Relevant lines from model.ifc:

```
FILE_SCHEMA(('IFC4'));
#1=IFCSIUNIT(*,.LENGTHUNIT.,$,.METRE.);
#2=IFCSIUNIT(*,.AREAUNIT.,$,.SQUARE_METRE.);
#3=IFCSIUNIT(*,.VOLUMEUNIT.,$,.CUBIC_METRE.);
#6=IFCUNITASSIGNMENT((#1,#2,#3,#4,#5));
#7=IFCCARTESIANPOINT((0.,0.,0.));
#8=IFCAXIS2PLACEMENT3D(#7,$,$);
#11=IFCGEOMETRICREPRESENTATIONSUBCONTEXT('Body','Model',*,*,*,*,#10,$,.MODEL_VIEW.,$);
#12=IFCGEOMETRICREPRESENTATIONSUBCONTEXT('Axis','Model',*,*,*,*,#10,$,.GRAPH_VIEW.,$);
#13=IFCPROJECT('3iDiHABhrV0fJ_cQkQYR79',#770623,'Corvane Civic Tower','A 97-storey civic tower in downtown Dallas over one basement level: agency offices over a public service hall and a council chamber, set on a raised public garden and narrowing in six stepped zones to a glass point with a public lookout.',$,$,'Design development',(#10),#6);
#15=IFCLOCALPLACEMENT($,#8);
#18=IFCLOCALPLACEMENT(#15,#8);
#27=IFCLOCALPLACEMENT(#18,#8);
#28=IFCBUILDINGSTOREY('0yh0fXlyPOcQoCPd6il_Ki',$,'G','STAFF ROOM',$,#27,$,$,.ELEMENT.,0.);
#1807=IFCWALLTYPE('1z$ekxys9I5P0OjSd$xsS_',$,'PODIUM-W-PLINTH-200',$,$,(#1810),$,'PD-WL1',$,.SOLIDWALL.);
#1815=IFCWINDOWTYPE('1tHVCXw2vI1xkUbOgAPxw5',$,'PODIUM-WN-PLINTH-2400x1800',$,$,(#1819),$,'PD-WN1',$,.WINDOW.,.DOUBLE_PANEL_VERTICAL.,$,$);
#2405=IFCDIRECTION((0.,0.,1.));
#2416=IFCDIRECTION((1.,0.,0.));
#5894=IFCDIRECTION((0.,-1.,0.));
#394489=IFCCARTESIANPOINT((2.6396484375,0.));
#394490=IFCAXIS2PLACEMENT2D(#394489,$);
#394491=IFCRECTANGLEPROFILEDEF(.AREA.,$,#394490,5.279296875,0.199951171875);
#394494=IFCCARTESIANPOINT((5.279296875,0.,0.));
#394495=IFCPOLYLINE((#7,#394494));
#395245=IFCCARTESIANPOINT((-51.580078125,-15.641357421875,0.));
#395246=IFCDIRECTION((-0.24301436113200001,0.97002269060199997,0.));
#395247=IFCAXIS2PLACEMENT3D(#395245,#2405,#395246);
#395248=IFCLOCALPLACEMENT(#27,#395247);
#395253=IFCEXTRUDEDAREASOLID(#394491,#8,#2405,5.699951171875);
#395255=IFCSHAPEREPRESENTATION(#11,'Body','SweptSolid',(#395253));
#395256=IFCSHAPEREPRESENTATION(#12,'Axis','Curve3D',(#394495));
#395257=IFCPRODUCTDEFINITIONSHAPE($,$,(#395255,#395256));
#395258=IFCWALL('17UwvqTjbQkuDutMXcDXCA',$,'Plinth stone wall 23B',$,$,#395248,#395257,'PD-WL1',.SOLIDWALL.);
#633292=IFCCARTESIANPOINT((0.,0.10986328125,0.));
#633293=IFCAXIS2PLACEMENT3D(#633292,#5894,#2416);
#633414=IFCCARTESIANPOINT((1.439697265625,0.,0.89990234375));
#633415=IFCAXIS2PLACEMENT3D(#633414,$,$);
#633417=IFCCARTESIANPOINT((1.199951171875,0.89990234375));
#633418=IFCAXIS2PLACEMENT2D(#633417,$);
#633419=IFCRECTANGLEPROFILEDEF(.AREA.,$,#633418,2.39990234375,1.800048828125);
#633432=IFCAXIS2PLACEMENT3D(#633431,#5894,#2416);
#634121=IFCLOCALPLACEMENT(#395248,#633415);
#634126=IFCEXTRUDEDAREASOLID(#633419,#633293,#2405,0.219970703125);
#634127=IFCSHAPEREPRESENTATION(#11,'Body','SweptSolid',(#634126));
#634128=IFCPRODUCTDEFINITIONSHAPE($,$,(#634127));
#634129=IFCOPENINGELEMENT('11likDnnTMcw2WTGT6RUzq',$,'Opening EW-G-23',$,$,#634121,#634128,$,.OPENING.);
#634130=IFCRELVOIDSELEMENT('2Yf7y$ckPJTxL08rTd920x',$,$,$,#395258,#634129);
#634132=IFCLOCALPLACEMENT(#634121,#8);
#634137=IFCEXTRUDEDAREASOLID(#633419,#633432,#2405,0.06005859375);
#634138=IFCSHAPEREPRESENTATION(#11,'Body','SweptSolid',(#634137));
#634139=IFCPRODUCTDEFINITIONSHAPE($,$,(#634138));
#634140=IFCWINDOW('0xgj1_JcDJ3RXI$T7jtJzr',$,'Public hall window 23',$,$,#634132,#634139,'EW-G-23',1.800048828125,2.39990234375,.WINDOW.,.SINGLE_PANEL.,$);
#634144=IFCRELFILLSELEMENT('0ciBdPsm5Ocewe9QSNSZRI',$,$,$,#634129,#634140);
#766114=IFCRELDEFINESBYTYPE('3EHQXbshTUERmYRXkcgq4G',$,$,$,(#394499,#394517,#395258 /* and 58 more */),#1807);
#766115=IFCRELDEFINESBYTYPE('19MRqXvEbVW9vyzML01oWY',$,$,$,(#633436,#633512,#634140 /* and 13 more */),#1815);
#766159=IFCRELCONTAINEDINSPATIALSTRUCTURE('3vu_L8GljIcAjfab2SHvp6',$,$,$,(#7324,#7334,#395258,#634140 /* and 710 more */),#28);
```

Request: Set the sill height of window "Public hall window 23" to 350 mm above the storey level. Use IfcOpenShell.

```python
import numpy as np
import ifcopenshell
import ifcopenshell.api.geometry
import ifcopenshell.geom
import ifcopenshell.util.element
import ifcopenshell.util.placement
import ifcopenshell.util.shape
import ifcopenshell.util.unit

model = ifcopenshell.open("model.ifc")
unit_scale = ifcopenshell.util.unit.calculate_unit_scale(model)

window = model.by_guid("0xgj1_JcDJ3RXI$T7jtJzr")
opening = window.FillsVoids[0].RelatingOpeningElement
storey = ifcopenshell.util.element.get_container(window, ifc_class="IfcBuildingStorey")
level = ifcopenshell.util.placement.get_local_placement(storey.ObjectPlacement)[2, 3]

# The opening's origin need not be at the sill, so measure its lowest point.
shape = ifcopenshell.geom.create_shape(ifcopenshell.geom.settings(), opening)
bottom = ifcopenshell.util.shape.get_shape_bottom_elevation(shape, shape.geometry) / unit_scale
dz = level + 0.35 - bottom

shift = np.array([0.0, 0.0, dz])
# The window is placed relative to its opening, so it follows when the opening moves.
matrix = ifcopenshell.util.placement.get_local_placement(opening.ObjectPlacement)
matrix[:3, 3] += shift
ifcopenshell.api.geometry.edit_object_placement(
    model, product=opening, matrix=matrix, is_si=False, should_transform_children=True
)

print(f"moved by {dz * unit_scale:+.3f} m")

model.write("model_edited.ifc")
```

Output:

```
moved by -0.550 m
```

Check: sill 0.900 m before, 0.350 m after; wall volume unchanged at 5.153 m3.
